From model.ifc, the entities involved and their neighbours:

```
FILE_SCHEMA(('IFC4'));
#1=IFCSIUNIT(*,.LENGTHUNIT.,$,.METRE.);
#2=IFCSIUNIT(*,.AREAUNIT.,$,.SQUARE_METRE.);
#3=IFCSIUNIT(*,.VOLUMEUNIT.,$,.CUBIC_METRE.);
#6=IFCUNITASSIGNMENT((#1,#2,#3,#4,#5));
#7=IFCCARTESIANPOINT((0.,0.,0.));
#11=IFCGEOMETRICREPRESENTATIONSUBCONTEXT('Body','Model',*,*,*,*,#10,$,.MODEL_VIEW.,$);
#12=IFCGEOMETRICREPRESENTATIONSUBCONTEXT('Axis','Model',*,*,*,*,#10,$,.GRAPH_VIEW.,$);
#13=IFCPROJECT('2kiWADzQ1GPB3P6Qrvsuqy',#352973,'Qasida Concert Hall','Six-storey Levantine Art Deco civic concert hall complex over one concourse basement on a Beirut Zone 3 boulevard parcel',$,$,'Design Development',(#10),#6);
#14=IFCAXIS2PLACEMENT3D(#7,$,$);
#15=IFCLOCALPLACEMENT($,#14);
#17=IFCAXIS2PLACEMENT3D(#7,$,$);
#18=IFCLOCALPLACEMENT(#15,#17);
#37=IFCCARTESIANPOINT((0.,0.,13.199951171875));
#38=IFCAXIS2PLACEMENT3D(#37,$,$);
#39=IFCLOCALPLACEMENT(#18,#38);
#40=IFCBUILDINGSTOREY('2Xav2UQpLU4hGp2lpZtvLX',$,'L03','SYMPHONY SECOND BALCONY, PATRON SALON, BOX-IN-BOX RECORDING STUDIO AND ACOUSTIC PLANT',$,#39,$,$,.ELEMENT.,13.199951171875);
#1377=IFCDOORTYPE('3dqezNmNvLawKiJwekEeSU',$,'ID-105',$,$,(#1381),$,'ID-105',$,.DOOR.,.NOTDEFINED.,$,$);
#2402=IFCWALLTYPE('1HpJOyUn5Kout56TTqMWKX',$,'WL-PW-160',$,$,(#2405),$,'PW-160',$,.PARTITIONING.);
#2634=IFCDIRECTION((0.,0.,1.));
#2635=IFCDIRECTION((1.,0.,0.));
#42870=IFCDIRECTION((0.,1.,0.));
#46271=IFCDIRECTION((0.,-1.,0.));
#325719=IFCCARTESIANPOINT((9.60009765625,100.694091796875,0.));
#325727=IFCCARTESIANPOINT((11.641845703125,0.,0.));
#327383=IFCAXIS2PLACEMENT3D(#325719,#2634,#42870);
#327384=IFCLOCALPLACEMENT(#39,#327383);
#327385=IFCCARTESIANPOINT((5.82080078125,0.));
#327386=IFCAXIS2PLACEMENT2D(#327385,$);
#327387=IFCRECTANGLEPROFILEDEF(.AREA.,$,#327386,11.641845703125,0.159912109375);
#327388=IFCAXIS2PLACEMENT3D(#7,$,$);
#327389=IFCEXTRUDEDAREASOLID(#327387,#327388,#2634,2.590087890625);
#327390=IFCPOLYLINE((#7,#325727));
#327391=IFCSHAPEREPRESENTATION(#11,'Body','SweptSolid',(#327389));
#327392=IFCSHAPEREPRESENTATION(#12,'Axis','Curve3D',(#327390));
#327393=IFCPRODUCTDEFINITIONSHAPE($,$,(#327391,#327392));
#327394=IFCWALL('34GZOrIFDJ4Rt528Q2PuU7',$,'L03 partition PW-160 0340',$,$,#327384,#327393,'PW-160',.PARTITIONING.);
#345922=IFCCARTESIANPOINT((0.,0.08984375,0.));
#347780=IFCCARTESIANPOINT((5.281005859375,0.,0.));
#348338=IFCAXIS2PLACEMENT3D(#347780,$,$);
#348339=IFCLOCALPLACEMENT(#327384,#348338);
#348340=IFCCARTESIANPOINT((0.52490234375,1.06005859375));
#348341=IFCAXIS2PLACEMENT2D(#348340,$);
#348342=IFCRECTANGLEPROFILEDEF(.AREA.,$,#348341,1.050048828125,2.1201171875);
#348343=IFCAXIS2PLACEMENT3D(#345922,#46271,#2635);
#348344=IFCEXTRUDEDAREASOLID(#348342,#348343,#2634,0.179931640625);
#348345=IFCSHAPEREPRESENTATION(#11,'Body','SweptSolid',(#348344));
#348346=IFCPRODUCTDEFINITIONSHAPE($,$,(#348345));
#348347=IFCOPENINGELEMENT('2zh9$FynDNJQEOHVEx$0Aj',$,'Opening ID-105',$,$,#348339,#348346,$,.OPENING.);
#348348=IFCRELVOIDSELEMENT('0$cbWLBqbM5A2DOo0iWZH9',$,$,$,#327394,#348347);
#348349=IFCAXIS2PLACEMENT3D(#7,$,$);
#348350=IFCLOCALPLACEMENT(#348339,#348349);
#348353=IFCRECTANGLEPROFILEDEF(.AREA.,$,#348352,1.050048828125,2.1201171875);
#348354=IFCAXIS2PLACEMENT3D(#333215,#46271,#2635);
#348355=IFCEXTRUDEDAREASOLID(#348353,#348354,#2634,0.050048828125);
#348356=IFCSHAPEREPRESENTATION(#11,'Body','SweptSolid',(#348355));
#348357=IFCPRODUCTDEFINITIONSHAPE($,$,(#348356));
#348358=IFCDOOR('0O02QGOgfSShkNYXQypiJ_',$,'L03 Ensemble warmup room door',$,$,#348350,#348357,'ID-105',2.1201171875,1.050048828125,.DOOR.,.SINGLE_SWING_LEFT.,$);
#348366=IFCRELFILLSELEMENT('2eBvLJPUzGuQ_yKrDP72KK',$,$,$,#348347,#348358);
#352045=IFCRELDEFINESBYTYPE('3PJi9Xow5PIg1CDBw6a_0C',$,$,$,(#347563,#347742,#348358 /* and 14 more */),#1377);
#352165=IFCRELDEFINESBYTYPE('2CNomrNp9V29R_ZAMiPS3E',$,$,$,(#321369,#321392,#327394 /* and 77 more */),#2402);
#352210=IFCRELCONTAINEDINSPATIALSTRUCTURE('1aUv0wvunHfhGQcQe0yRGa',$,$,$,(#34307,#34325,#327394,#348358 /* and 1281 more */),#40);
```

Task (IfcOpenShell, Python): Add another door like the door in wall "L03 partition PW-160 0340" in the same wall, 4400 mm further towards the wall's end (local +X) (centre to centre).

```python
import ifcopenshell
import ifcopenshell.api.feature
import ifcopenshell.api.geometry
import ifcopenshell.api.root
import ifcopenshell.geom
import ifcopenshell.util.element
import ifcopenshell.util.placement
import ifcopenshell.util.shape

model = ifcopenshell.open("model.ifc")
settings = ifcopenshell.geom.settings()


def volume(element):
    """Net volume in cubic metres, openings subtracted."""
    shape = ifcopenshell.geom.create_shape(settings, element)
    return ifcopenshell.util.shape.get_volume(shape.geometry)


door = model.by_guid("0O02QGOgfSShkNYXQypiJ_")
opening = door.FillsVoids[0].RelatingOpeningElement
wall = opening.VoidsElements[0].RelatingBuildingElement
before = volume(wall)
shift = ifcopenshell.util.placement.get_local_placement(wall.ObjectPlacement)[:3, 0] * 4.4

# copy_class copies the void relationship, type, container and properties, but no geometry.
new_opening = ifcopenshell.api.root.copy_class(model, product=opening)
new_opening.Representation = ifcopenshell.util.element.copy_deep(
    model, opening.Representation, exclude=["IfcGeometricRepresentationContext", "IfcRepresentationMap"]
)
new_door = ifcopenshell.api.root.copy_class(model, product=door)
new_door.Representation = ifcopenshell.util.element.copy_deep(
    model, door.Representation, exclude=["IfcGeometricRepresentationContext", "IfcRepresentationMap"]
)
new_door.Tag = None
ifcopenshell.api.feature.add_filling(model, opening=new_opening, element=new_door)

for old, new in ((opening, new_opening), (door, new_door)):
    matrix = ifcopenshell.util.placement.get_local_placement(old.ObjectPlacement)
    matrix[:3, 3] += shift
    ifcopenshell.api.geometry.edit_object_placement(model, product=new, matrix=matrix, is_si=False)

after = volume(wall)

print(f"wall volume {before:.3f} -> {after:.3f} m3")

model.write("model_updated.ifc")
```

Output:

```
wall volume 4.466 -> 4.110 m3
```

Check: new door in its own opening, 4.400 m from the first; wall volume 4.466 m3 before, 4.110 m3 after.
